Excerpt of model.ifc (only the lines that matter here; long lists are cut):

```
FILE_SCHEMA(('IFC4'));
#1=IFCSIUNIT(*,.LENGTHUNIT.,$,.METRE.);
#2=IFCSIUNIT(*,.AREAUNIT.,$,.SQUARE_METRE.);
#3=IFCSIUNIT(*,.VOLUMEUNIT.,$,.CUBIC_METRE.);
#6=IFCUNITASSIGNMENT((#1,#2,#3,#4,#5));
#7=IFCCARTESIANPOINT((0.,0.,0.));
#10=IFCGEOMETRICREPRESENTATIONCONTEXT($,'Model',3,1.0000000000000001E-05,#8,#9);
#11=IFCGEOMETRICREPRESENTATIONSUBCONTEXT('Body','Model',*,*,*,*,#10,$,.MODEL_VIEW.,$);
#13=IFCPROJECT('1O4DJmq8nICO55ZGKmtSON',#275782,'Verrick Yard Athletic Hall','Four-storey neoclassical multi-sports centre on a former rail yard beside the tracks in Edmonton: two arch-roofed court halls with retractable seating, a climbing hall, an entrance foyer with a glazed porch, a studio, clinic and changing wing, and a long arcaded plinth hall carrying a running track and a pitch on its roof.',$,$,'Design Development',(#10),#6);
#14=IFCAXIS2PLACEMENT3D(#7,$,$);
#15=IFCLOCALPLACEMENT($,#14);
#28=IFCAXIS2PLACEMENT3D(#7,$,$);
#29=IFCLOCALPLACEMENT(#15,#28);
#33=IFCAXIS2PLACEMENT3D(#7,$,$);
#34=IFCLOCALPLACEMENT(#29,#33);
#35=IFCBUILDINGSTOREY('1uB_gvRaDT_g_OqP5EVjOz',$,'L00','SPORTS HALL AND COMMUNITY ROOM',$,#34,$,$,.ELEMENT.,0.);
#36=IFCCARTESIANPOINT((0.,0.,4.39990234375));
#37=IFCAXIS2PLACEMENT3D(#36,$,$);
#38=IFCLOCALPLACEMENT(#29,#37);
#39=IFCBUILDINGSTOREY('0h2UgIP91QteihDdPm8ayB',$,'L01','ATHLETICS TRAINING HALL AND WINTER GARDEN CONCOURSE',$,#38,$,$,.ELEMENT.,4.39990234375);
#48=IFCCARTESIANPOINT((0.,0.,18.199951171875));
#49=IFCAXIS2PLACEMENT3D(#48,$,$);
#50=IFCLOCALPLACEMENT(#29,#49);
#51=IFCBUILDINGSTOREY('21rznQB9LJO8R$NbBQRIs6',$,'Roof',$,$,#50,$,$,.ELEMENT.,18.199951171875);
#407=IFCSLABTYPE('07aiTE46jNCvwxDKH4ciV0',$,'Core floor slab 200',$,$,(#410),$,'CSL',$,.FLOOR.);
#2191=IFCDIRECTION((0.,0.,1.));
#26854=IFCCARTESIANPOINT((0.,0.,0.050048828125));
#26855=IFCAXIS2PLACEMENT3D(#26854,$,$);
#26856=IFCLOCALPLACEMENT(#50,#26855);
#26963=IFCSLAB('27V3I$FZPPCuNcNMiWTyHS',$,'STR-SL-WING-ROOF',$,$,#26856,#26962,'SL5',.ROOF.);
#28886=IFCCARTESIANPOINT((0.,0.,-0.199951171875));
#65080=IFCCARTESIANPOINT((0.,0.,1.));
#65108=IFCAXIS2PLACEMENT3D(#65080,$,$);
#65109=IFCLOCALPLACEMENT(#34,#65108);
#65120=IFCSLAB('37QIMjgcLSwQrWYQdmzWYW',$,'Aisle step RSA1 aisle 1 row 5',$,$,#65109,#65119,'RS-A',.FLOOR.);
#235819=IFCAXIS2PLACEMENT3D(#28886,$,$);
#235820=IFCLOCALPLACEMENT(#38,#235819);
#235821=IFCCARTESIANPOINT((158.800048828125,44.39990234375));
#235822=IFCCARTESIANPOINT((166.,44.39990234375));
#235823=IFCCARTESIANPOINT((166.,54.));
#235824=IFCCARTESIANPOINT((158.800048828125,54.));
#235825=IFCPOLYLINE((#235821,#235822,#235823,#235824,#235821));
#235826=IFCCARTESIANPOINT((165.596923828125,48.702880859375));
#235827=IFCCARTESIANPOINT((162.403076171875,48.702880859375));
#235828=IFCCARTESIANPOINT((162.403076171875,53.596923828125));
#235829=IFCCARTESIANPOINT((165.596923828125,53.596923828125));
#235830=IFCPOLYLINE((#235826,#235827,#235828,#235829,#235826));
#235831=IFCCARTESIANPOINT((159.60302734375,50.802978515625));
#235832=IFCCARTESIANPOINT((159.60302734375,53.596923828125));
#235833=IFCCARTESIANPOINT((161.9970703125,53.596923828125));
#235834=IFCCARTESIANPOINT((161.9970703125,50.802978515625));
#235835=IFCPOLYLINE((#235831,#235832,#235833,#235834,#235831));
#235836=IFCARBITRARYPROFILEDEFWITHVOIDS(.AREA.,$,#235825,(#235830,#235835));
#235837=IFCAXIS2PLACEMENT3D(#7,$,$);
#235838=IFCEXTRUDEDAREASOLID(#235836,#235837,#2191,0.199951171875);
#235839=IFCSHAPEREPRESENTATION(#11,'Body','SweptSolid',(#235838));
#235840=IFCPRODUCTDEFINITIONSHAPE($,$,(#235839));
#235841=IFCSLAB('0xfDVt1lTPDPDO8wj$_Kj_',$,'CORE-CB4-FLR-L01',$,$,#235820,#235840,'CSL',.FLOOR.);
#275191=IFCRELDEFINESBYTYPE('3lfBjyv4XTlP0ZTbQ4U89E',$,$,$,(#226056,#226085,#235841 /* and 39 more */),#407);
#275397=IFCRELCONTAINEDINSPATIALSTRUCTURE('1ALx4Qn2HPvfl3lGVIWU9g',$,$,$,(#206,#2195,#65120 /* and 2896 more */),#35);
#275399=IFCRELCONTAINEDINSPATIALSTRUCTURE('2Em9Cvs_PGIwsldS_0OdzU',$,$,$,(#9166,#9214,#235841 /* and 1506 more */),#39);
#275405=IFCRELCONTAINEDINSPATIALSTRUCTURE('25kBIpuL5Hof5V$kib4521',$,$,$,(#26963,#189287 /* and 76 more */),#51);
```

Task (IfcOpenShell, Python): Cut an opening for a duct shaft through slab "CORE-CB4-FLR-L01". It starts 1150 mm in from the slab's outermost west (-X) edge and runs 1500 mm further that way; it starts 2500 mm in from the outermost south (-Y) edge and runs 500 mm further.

```python
import numpy as np
import ifcopenshell
import ifcopenshell.api.feature
import ifcopenshell.api.geometry
import ifcopenshell.api.root
import ifcopenshell.geom
import ifcopenshell.util.placement
import ifcopenshell.util.representation
import ifcopenshell.util.shape
import ifcopenshell.util.unit

model = ifcopenshell.open("model.ifc")
unit_scale = ifcopenshell.util.unit.calculate_unit_scale(model)
settings = ifcopenshell.geom.settings()


def volume(element):
    """Net volume in cubic metres, openings subtracted."""
    shape = ifcopenshell.geom.create_shape(settings, element)
    return ifcopenshell.util.shape.get_volume(shape.geometry)


slab = model.by_guid("0xfDVt1lTPDPDO8wj$_Kj_")
before = volume(slab)

# Extent in the slab's own axes, in metres. The edges named are its -X and -Y sides.
slab_shape = ifcopenshell.geom.create_shape(settings, slab)
vertices = ifcopenshell.util.shape.get_vertices(slab_shape.geometry)
x_min, y_min, bottom = vertices.min(axis=0)
top = vertices[:, 2].max()

opening = ifcopenshell.api.root.create_entity(model, ifc_class="IfcOpeningElement", name="Duct shaft opening", predefined_type="OPENING")
context = ifcopenshell.util.representation.get_context(model, "Model", "Body", "MODEL_VIEW")
width, depth = 1.5, 0.5
outline = [(0.0, 0.0), (width, 0.0), (width, depth), (0.0, depth), (0.0, 0.0)]
# Overshoot both faces by 50 mm so the cut is clean.
shape = ifcopenshell.api.geometry.add_slab_representation(
    model, context=context, depth=top - bottom + 0.1, polyline=outline
)
ifcopenshell.api.geometry.assign_representation(model, product=opening, representation=shape)

matrix = ifcopenshell.util.placement.get_local_placement(slab.ObjectPlacement)
matrix[:, 3] = matrix @ np.append(np.array([x_min + 1.15, y_min + 2.5, bottom - 0.05]) / unit_scale, 1.0)
ifcopenshell.api.geometry.edit_object_placement(model, product=opening, matrix=matrix, is_si=False)
ifcopenshell.api.feature.add_feature(model, feature=opening, element=slab)

after = volume(slab)

print(f"slab volume {before:.3f} -> {after:.3f} m3")

model.write("model-out.ifc")
```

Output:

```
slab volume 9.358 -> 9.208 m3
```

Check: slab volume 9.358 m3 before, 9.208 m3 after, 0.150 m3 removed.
